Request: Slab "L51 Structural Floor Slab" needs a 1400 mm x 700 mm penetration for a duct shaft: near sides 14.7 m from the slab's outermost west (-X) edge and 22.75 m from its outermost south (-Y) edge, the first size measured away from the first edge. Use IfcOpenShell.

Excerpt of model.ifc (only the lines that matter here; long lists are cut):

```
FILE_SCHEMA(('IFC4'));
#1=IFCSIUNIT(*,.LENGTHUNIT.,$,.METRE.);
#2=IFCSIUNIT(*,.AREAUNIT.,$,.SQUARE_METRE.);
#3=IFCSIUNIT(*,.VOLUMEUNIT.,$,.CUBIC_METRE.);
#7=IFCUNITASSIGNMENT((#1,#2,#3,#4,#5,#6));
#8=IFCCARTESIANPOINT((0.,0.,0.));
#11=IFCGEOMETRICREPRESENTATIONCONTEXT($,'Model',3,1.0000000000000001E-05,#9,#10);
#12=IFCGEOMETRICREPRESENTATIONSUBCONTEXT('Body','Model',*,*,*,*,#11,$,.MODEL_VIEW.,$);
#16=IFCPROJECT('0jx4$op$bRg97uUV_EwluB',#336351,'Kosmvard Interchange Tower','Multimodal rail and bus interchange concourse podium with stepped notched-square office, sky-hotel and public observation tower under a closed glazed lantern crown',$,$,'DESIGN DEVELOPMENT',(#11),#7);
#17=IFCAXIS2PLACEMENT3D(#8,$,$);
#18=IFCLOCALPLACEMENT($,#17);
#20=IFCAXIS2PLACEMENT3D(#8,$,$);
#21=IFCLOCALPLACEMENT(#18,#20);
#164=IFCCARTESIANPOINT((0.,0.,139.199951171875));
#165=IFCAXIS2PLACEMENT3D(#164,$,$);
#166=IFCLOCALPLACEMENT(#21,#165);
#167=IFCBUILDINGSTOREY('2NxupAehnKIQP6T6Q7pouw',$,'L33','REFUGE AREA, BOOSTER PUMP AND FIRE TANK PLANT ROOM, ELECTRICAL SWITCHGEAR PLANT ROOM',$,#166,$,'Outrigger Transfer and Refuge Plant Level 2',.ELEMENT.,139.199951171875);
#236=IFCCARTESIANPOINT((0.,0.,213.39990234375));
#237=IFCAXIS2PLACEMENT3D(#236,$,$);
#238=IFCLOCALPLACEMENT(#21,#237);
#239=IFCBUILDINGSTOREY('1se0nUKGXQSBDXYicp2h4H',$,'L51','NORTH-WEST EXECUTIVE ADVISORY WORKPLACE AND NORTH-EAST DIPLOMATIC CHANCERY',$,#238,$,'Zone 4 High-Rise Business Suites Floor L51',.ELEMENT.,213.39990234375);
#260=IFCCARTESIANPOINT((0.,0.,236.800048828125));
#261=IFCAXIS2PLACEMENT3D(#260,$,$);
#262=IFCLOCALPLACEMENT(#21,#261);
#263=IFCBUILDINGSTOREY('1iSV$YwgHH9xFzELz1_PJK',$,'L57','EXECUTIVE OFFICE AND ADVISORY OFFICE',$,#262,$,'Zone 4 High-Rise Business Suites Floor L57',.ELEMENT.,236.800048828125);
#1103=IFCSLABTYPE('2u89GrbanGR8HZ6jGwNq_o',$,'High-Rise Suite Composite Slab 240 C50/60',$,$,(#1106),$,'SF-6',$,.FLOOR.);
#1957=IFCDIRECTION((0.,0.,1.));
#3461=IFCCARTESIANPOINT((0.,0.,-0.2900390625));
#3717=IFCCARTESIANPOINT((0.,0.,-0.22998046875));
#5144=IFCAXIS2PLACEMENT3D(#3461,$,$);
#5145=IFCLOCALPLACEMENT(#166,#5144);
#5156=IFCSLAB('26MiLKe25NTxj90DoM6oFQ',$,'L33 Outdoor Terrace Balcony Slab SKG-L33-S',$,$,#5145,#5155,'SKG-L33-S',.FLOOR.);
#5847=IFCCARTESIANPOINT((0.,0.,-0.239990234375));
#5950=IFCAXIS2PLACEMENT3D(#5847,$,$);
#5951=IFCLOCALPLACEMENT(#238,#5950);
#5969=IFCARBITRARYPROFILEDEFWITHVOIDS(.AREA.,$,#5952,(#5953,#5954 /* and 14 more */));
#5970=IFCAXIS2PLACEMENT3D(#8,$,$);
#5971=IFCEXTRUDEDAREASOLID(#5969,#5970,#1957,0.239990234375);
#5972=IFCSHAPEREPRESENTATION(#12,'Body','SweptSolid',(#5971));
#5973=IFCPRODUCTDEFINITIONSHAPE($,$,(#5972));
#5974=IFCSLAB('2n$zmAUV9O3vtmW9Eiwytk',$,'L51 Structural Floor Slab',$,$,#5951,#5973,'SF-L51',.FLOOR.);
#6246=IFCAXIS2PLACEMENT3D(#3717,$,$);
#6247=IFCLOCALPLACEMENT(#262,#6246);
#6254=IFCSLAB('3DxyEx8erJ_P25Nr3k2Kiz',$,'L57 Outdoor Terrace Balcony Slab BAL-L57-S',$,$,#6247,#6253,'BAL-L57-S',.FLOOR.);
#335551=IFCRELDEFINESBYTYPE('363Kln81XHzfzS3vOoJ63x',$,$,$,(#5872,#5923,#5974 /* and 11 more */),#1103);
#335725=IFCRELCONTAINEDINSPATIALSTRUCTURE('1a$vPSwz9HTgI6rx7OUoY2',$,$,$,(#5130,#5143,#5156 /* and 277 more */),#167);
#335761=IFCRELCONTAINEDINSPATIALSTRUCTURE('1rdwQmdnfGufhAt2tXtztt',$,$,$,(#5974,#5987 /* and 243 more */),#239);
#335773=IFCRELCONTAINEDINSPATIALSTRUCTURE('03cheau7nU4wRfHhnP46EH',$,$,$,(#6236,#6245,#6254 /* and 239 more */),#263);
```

```python
import numpy as np
import ifcopenshell
import ifcopenshell.api.feature
import ifcopenshell.api.geometry
import ifcopenshell.api.root
import ifcopenshell.geom
import ifcopenshell.util.placement
import ifcopenshell.util.representation
import ifcopenshell.util.shape
import ifcopenshell.util.unit

model = ifcopenshell.open("model.ifc")
unit_scale = ifcopenshell.util.unit.calculate_unit_scale(model)
settings = ifcopenshell.geom.settings()


def volume(element):
    """Net volume in cubic metres, openings subtracted."""
    shape = ifcopenshell.geom.create_shape(settings, element)
    return ifcopenshell.util.shape.get_volume(shape.geometry)


slab = model.by_id(5974)
before = volume(slab)

# Extent in the slab's own axes, in metres. The edges named are its -X and -Y sides.
slab_shape = ifcopenshell.geom.create_shape(settings, slab)
vertices = ifcopenshell.util.shape.get_vertices(slab_shape.geometry)
x_min, y_min, bottom = vertices.min(axis=0)
top = vertices[:, 2].max()

opening = ifcopenshell.api.root.create_entity(model, ifc_class="IfcOpeningElement", name="Duct shaft opening", predefined_type="OPENING")
context = ifcopenshell.util.representation.get_context(model, "Model", "Body", "MODEL_VIEW")
width, depth = 1.4, 0.7
outline = [(0.0, 0.0), (width, 0.0), (width, depth), (0.0, depth), (0.0, 0.0)]
# Overshoot both faces by 50 mm so the cut is clean.
shape = ifcopenshell.api.geometry.add_slab_representation(
    model, context=context, depth=top - bottom + 0.1, polyline=outline
)
ifcopenshell.api.geometry.assign_representation(model, product=opening, representation=shape)

matrix = ifcopenshell.util.placement.get_local_placement(slab.ObjectPlacement)
matrix[:, 3] = matrix @ np.append(np.array([x_min + 14.7, y_min + 22.75, bottom - 0.05]) / unit_scale, 1.0)
ifcopenshell.api.geometry.edit_object_placement(model, product=opening, matrix=matrix, is_si=False)
ifcopenshell.api.feature.add_feature(model, feature=opening, element=slab)

after = volume(slab)

print(f"slab volume {before:.3f} -> {after:.3f} m3")

model.write("model_updated.ifc")
```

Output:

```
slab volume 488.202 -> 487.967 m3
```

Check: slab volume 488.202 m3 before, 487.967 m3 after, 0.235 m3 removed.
